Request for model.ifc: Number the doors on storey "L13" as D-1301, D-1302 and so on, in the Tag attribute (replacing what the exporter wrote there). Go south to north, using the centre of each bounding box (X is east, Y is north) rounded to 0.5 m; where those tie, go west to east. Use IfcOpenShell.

First a look at what the model holds.

```python
import ifcopenshell
import ifcopenshell.util.element
import ifcopenshell.util.placement

model = ifcopenshell.open("model.ifc")
print(model.schema)
storey = next(s for s in model.by_type("IfcBuildingStorey") if s.Name == "L13")
doors = [e for e in ifcopenshell.util.element.get_decomposition(storey) if e.is_a("IfcDoor")]
for e in sorted(doors, key=lambda e: e.id()):
    origin = ifcopenshell.util.placement.get_local_placement(e.ObjectPlacement)[:3, 3]
    print(e.id(), e.Tag, e.Name, origin.round(2) + 0.0, sep=" | ")
```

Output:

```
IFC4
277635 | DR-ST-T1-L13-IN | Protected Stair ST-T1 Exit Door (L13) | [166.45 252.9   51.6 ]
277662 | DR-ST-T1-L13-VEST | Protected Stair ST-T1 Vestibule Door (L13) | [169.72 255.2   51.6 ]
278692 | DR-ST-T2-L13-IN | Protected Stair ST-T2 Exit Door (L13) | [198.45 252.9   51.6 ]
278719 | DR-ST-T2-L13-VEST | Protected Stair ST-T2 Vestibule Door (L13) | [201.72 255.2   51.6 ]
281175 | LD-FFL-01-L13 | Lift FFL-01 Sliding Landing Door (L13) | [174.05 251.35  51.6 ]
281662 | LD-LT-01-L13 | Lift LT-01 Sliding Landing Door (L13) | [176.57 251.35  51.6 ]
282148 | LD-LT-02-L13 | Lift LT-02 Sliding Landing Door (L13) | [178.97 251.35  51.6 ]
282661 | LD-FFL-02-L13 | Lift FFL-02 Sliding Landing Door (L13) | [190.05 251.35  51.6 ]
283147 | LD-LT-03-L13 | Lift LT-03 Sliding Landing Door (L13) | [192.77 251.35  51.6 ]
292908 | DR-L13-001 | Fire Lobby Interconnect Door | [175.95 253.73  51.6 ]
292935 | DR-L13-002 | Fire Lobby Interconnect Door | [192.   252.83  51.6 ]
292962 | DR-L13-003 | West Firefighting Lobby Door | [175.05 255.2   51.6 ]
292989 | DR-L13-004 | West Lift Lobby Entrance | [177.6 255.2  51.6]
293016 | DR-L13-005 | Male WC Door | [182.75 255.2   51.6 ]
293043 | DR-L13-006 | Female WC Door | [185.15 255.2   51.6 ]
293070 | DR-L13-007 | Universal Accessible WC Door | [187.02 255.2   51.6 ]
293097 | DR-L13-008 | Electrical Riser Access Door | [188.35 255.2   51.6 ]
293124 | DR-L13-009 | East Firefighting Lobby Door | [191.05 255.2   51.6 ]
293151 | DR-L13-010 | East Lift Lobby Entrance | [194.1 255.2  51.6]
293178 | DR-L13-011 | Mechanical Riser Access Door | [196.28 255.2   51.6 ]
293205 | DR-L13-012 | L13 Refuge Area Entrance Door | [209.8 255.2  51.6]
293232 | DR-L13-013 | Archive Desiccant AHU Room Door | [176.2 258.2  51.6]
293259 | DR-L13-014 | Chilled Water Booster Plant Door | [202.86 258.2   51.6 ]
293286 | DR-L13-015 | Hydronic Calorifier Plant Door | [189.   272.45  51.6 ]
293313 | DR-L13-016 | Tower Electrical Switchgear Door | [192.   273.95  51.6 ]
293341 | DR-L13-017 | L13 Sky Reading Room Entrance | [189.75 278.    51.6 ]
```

```python
import ifcopenshell
import ifcopenshell.geom
import ifcopenshell.util.element
import ifcopenshell.util.shape

model = ifcopenshell.open("model.ifc")
settings = ifcopenshell.geom.settings()
settings.set("use-world-coords", True)


def centre(element):
    shape = ifcopenshell.geom.create_shape(settings, element)
    return ifcopenshell.util.shape.get_bbox_centroid(shape.geometry)


storey = next(s for s in model.by_type("IfcBuildingStorey") if s.Name == "L13")
doors = [e for e in ifcopenshell.util.element.get_decomposition(storey) if e.is_a("IfcDoor")]

# Insertion points can sit at a corner or the storey origin, so sort by the geometry (in metres).
centres = {e: centre(e) for e in doors}
doors.sort(key=lambda e: (round(centres[e][1] / 0.5), centres[e][0]))

for i, e in enumerate(doors, start=1):
    number = f"D-13{i:02d}"
    e.Tag = number
    print(e.id(), number)

model.write("model-out.ifc")
```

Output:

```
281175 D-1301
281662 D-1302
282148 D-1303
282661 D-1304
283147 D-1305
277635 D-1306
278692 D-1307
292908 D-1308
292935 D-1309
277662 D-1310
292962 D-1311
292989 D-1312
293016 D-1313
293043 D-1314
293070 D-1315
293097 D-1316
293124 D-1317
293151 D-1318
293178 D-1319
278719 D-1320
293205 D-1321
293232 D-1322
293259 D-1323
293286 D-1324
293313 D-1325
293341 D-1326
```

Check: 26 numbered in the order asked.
